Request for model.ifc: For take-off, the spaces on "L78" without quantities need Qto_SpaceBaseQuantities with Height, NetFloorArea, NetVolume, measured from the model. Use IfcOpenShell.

First a look at what the model holds.

```python
import ifcopenshell
import ifcopenshell.util.element
import ifcopenshell.util.unit

model = ifcopenshell.open("model.ifc")
print(model.schema)
for unit_type in ("LENGTHUNIT", "AREAUNIT", "VOLUMEUNIT"):
    print(unit_type, ifcopenshell.util.unit.calculate_unit_scale(model, unit_type))
storey = next(s for s in model.by_type("IfcBuildingStorey") if s.Name == "L78")
spaces = [e for e in ifcopenshell.util.element.get_decomposition(storey) if e.is_a("IfcSpace")]
for e in sorted(spaces, key=lambda e: e.id()):
    print(e.id(), e.is_a(), e.Name, list(ifcopenshell.util.element.get_psets(e, qtos_only=True)), sep=" | ")
```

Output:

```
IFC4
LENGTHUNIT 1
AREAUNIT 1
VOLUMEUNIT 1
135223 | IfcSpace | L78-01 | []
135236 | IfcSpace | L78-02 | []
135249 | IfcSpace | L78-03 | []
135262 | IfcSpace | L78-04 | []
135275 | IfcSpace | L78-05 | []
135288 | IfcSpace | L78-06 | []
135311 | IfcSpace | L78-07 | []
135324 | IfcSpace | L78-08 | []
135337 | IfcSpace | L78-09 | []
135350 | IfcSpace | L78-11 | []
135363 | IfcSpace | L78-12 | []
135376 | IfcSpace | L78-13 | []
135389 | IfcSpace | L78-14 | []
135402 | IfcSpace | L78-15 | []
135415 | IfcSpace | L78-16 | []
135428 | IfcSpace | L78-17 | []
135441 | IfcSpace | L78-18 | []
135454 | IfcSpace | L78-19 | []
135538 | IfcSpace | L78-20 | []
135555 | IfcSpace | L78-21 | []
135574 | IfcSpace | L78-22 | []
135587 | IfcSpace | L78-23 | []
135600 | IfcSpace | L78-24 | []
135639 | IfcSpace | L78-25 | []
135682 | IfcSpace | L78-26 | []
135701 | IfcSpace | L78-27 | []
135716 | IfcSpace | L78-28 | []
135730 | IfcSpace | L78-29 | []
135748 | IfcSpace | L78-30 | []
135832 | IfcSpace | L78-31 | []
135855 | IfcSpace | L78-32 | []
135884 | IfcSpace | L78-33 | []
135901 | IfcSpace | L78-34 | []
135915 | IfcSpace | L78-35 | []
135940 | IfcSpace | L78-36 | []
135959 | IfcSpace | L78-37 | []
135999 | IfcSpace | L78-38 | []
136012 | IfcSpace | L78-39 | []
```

```python
import ifcopenshell
import ifcopenshell.api.pset
import ifcopenshell.geom
import ifcopenshell.util.element
import ifcopenshell.util.shape
import ifcopenshell.util.unit

model = ifcopenshell.open("model.ifc")
unit_scale = ifcopenshell.util.unit.calculate_unit_scale(model)
area_scale = ifcopenshell.util.unit.calculate_unit_scale(model, "AREAUNIT")
volume_scale = ifcopenshell.util.unit.calculate_unit_scale(model, "VOLUMEUNIT")
settings = ifcopenshell.geom.settings()

storey = next(s for s in model.by_type("IfcBuildingStorey") if s.Name == "L78")
spaces = [e for e in ifcopenshell.util.element.get_decomposition(storey) if e.is_a("IfcSpace")]

for e in sorted(spaces, key=lambda e: e.id()):
    if ifcopenshell.util.element.get_psets(e, qtos_only=True, should_inherit=False):
        continue
    # Geometry comes back in metres, in the element's own axes.
    shape = ifcopenshell.geom.create_shape(settings, e)
    values = {
        "Height": ifcopenshell.util.shape.get_z(shape.geometry) / unit_scale,
        "NetFloorArea": ifcopenshell.util.shape.get_footprint_area(shape.geometry) / area_scale,
        "NetVolume": ifcopenshell.util.shape.get_volume(shape.geometry) / volume_scale,
    }
    qto = ifcopenshell.api.pset.add_qto(model, product=e, name="Qto_SpaceBaseQuantities")
    ifcopenshell.api.pset.edit_qto(model, qto=qto, properties=values)
    print(e.id(), {k: round(v, 3) for k, v in values.items()})

model.write("model_v2.ifc")
```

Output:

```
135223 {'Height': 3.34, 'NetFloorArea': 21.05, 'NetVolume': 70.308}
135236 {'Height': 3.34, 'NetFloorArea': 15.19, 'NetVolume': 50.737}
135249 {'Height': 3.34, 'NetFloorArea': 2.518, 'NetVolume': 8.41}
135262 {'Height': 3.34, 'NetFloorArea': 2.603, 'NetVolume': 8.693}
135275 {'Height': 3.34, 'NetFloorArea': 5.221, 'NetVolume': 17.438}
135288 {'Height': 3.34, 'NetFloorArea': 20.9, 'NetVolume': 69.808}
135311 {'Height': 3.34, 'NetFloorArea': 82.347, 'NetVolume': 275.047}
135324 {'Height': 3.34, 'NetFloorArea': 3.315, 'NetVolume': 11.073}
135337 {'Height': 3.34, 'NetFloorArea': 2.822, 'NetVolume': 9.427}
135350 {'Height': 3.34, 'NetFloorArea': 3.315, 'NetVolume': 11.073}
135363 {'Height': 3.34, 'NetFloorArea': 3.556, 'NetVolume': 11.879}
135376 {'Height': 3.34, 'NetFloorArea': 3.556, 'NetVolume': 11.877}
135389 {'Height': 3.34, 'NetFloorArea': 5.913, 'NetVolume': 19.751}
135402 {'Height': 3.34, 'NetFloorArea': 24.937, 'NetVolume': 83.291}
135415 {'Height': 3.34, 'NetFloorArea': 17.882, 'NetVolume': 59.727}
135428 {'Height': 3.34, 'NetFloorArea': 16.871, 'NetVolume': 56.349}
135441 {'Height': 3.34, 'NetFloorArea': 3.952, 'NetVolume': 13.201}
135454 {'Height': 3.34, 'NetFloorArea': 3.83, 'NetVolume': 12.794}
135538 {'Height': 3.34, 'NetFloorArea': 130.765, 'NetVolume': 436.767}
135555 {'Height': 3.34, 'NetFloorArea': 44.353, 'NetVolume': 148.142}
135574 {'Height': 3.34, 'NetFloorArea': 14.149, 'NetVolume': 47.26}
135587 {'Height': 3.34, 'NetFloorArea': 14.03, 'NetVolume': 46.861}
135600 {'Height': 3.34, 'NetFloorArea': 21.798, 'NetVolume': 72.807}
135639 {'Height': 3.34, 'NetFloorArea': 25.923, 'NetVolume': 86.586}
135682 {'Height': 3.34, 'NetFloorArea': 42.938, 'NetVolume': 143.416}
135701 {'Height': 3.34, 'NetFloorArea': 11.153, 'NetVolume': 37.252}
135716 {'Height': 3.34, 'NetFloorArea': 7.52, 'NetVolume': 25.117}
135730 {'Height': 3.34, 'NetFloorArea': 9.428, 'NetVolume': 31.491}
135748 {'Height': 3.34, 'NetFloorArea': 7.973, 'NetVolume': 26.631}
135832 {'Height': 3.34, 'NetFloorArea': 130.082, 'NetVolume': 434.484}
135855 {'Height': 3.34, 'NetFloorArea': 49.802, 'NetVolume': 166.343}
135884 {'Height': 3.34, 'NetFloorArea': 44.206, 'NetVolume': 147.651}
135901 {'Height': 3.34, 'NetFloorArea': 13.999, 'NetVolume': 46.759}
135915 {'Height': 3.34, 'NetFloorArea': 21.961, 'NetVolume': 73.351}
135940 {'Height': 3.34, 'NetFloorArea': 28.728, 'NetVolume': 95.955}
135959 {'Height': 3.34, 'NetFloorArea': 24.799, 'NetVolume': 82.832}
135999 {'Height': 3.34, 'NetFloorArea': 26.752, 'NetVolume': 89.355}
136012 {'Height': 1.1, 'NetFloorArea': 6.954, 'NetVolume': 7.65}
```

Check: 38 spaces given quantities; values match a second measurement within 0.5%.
